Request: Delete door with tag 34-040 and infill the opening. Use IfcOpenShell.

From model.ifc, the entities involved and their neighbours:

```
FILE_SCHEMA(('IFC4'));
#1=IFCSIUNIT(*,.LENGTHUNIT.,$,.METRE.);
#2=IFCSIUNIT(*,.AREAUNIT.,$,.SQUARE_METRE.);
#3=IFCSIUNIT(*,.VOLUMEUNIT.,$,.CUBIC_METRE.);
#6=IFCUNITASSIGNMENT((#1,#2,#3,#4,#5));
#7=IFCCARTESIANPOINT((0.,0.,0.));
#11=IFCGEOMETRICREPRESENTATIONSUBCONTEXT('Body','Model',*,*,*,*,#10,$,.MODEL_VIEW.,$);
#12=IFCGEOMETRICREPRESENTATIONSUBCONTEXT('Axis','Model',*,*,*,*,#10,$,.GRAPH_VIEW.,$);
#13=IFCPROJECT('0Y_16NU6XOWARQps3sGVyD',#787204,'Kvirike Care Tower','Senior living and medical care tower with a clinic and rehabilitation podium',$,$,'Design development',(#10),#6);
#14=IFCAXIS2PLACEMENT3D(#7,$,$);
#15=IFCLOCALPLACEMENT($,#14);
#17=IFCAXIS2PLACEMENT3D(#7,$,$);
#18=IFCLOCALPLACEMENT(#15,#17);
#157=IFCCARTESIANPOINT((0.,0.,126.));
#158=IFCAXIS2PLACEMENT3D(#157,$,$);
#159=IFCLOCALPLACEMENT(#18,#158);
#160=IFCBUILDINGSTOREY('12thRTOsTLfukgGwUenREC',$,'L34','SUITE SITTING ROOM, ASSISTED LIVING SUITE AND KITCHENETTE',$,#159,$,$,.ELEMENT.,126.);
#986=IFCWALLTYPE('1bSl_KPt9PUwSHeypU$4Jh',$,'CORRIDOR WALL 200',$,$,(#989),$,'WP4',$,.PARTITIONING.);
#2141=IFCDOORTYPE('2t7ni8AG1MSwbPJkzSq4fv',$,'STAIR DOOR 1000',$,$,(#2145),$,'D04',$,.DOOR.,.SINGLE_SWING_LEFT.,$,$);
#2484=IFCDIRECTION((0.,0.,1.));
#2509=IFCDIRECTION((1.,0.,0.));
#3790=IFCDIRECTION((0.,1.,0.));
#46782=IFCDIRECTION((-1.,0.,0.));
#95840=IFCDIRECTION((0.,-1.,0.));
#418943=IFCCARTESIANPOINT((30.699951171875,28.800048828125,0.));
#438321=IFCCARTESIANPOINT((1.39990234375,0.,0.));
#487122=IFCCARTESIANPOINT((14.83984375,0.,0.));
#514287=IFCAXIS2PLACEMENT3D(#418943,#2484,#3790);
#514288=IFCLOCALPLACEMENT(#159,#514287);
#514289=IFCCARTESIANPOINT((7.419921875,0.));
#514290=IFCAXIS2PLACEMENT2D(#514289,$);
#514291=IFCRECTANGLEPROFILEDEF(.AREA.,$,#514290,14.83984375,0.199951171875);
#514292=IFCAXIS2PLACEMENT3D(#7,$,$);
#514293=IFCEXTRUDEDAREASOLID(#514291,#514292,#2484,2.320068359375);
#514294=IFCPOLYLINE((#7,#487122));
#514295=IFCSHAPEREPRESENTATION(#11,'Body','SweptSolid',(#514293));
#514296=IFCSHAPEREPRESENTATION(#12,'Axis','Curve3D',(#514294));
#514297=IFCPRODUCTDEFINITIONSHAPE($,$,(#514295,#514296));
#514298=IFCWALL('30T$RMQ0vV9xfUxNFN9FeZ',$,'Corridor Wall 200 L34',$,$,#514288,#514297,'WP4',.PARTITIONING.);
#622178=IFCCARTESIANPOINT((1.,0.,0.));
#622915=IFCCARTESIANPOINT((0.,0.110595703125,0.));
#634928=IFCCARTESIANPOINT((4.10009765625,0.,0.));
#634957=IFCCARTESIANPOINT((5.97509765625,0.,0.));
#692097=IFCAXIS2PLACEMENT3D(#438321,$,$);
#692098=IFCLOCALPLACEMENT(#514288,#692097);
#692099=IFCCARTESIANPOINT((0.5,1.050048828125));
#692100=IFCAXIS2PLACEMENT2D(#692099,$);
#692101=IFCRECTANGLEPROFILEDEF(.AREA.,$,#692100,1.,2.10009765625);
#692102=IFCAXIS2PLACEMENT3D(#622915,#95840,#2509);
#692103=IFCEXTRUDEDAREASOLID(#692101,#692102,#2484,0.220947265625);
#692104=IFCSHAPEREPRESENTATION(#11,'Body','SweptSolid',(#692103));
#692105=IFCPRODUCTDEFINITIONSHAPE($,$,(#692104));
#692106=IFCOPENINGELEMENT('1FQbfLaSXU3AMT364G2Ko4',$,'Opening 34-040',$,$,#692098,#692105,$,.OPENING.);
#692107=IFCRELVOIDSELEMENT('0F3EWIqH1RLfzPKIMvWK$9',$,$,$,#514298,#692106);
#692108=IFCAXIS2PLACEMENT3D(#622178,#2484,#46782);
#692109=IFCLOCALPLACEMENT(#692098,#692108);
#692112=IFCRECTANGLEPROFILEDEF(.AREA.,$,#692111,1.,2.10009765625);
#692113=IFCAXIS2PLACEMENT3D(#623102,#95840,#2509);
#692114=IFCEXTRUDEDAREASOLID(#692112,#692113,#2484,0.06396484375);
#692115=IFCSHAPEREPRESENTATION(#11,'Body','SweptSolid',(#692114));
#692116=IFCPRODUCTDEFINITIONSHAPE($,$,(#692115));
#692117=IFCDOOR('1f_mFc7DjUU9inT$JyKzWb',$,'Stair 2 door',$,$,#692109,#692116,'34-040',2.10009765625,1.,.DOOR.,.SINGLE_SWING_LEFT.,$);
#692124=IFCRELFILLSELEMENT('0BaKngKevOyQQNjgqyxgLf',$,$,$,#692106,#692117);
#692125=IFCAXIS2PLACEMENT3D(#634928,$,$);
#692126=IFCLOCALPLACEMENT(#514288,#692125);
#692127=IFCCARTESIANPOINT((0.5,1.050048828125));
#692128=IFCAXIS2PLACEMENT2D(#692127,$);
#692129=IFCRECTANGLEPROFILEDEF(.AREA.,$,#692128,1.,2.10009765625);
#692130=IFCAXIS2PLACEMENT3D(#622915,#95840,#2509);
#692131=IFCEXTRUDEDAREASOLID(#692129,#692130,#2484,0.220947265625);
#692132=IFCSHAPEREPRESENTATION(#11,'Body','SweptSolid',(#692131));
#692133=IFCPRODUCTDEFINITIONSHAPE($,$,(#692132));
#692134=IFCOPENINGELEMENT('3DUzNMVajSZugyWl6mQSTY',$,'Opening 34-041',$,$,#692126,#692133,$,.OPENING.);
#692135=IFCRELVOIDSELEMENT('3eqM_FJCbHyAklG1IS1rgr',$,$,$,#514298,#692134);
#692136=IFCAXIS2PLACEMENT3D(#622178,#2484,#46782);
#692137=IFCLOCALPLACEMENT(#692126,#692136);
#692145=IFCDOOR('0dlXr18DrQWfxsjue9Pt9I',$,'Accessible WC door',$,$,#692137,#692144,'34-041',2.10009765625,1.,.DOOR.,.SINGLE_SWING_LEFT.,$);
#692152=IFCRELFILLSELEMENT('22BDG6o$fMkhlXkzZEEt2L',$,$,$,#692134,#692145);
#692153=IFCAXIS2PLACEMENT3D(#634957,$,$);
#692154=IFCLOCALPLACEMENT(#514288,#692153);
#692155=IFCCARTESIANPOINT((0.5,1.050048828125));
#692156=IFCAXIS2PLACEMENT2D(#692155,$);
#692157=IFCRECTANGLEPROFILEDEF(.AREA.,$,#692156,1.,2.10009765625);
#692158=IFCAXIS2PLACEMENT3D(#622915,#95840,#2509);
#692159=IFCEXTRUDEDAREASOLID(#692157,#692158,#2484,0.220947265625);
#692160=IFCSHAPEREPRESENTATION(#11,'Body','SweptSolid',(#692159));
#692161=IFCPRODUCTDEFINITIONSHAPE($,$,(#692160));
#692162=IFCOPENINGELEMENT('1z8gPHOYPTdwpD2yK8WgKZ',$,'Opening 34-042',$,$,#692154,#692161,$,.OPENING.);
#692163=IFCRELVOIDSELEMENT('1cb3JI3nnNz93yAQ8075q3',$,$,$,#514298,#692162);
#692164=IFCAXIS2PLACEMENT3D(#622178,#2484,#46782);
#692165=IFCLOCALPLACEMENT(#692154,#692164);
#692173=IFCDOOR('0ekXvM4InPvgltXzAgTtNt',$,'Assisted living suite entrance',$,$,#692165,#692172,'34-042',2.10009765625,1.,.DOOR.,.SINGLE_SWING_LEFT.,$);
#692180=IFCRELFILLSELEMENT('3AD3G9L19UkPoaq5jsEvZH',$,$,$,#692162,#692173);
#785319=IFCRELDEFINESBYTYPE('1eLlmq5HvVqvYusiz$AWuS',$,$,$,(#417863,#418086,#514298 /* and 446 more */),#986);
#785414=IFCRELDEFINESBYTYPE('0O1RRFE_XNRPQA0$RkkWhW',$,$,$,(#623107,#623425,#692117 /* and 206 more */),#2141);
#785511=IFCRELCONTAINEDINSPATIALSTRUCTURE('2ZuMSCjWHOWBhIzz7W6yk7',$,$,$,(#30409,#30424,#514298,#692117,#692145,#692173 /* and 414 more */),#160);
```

```python
import ifcopenshell
import ifcopenshell.api.feature
import ifcopenshell.api.root
import ifcopenshell.geom
import ifcopenshell.util.shape

model = ifcopenshell.open("model.ifc")
settings = ifcopenshell.geom.settings()


def volume(element):
    """Net volume in cubic metres, openings subtracted."""
    shape = ifcopenshell.geom.create_shape(settings, element)
    return ifcopenshell.util.shape.get_volume(shape.geometry)


door = model.by_guid("1f_mFc7DjUU9inT$JyKzWb")
opening = door.FillsVoids[0].RelatingOpeningElement
wall = opening.VoidsElements[0].RelatingBuildingElement
before = volume(wall)

ifcopenshell.api.root.remove_product(model, product=door)
ifcopenshell.api.feature.remove_feature(model, feature=opening)

after = volume(wall)

print(f"wall volume {before:.3f} -> {after:.3f} m3")

model.write("model-out.ifc")
```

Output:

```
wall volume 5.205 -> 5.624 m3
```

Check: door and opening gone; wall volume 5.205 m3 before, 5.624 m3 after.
